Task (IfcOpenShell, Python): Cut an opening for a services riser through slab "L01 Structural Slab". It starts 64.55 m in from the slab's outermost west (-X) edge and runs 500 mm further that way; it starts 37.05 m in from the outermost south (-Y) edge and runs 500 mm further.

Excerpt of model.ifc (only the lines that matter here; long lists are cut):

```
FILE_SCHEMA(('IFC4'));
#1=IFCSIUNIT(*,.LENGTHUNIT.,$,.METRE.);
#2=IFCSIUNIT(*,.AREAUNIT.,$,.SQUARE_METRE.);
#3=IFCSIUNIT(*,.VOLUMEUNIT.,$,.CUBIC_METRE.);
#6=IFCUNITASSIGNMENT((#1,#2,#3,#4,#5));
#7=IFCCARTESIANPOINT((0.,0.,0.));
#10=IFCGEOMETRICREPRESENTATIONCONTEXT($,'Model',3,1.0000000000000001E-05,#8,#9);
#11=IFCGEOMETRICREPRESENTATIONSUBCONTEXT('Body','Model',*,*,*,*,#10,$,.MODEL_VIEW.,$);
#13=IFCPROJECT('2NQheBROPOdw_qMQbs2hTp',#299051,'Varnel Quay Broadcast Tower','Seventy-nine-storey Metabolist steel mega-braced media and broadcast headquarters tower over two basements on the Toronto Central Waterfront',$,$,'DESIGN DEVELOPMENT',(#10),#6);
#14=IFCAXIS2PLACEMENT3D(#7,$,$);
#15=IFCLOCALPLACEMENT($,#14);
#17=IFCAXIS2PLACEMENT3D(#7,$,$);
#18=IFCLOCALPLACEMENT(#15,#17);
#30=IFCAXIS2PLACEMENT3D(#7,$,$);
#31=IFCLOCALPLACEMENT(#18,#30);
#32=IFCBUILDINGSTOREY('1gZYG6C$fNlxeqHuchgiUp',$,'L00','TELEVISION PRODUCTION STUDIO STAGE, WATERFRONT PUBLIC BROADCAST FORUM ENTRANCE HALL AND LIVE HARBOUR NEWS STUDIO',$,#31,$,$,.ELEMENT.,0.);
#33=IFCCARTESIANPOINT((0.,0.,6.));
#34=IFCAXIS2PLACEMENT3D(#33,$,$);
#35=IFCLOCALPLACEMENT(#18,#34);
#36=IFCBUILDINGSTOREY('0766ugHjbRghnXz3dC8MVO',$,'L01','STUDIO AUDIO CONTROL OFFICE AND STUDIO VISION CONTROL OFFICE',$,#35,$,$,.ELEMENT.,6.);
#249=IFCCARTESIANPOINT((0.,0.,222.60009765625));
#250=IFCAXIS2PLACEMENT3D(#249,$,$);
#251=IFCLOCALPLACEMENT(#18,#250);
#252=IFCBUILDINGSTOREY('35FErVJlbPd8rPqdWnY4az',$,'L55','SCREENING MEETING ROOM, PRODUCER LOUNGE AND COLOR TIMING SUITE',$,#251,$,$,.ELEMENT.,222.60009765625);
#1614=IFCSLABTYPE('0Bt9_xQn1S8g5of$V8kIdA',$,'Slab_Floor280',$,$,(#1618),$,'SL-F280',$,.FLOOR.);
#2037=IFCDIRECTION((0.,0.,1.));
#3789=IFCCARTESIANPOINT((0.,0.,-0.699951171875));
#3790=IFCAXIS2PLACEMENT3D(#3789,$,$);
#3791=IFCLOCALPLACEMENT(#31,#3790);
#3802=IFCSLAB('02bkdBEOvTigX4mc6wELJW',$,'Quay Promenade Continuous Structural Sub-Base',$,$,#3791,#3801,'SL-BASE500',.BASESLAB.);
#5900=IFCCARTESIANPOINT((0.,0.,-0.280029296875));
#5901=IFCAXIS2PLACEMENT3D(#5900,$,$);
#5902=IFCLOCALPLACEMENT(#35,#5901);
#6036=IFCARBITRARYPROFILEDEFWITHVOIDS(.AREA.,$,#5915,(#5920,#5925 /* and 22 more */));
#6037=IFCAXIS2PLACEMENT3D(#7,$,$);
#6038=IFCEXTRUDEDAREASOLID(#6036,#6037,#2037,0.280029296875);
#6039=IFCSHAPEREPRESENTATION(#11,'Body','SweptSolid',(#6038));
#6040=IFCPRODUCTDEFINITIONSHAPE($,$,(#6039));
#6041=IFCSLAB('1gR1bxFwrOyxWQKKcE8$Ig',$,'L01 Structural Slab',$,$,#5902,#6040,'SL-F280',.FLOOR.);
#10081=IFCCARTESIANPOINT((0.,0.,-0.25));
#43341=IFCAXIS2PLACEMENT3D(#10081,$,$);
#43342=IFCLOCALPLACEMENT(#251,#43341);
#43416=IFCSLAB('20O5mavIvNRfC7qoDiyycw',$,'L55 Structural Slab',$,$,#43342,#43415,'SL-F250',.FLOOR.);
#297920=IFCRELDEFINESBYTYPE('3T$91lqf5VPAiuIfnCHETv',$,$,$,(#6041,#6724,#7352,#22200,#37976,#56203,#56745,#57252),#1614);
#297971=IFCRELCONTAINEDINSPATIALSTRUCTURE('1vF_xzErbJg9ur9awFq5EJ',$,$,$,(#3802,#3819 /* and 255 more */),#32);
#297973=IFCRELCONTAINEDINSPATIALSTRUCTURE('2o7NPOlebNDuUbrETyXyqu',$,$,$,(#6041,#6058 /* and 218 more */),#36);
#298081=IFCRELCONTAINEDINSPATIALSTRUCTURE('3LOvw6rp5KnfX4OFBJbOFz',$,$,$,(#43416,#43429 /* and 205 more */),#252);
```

```python
import numpy as np
import ifcopenshell
import ifcopenshell.api.feature
import ifcopenshell.api.geometry
import ifcopenshell.api.root
import ifcopenshell.geom
import ifcopenshell.util.placement
import ifcopenshell.util.representation
import ifcopenshell.util.shape
import ifcopenshell.util.unit

model = ifcopenshell.open("model.ifc")
unit_scale = ifcopenshell.util.unit.calculate_unit_scale(model)
settings = ifcopenshell.geom.settings()


def volume(element):
    """Net volume in cubic metres, openings subtracted."""
    shape = ifcopenshell.geom.create_shape(settings, element)
    return ifcopenshell.util.shape.get_volume(shape.geometry)


slab = model.by_guid("1gR1bxFwrOyxWQKKcE8$Ig")
before = volume(slab)

# Extent in the slab's own axes, in metres. The edges named are its -X and -Y sides.
slab_shape = ifcopenshell.geom.create_shape(settings, slab)
vertices = ifcopenshell.util.shape.get_vertices(slab_shape.geometry)
x_min, y_min, bottom = vertices.min(axis=0)
top = vertices[:, 2].max()

opening = ifcopenshell.api.root.create_entity(model, ifc_class="IfcOpeningElement", name="Services riser opening", predefined_type="OPENING")
context = ifcopenshell.util.representation.get_context(model, "Model", "Body", "MODEL_VIEW")
width, depth = 0.5, 0.5
outline = [(0.0, 0.0), (width, 0.0), (width, depth), (0.0, depth), (0.0, 0.0)]
# Overshoot both faces by 50 mm so the cut is clean.
shape = ifcopenshell.api.geometry.add_slab_representation(
    model, context=context, depth=top - bottom + 0.1, polyline=outline
)
ifcopenshell.api.geometry.assign_representation(model, product=opening, representation=shape)

matrix = ifcopenshell.util.placement.get_local_placement(slab.ObjectPlacement)
matrix[:, 3] = matrix @ np.append(np.array([x_min + 64.55, y_min + 37.05, bottom - 0.05]) / unit_scale, 1.0)
ifcopenshell.api.geometry.edit_object_placement(model, product=opening, matrix=matrix, is_si=False)
ifcopenshell.api.feature.add_feature(model, feature=opening, element=slab)

after = volume(slab)

print(f"slab volume {before:.3f} -> {after:.3f} m3")

model.write("model_edited.ifc")
```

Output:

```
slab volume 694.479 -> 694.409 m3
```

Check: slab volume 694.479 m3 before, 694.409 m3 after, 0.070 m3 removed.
